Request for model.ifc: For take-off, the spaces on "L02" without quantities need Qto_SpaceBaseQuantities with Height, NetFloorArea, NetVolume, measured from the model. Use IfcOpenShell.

First a look at what the model holds.

```python
import ifcopenshell
import ifcopenshell.util.element
import ifcopenshell.util.unit

model = ifcopenshell.open("model.ifc")
print(model.schema)
for unit_type in ("LENGTHUNIT", "AREAUNIT", "VOLUMEUNIT"):
    print(unit_type, ifcopenshell.util.unit.calculate_unit_scale(model, unit_type))
storey = next(s for s in model.by_type("IfcBuildingStorey") if s.Name == "L02")
spaces = [e for e in ifcopenshell.util.element.get_decomposition(storey) if e.is_a("IfcSpace")]
for e in sorted(spaces, key=lambda e: e.id()):
    print(e.id(), e.is_a(), e.Name, list(ifcopenshell.util.element.get_psets(e, qtos_only=True)), sep=" | ")
```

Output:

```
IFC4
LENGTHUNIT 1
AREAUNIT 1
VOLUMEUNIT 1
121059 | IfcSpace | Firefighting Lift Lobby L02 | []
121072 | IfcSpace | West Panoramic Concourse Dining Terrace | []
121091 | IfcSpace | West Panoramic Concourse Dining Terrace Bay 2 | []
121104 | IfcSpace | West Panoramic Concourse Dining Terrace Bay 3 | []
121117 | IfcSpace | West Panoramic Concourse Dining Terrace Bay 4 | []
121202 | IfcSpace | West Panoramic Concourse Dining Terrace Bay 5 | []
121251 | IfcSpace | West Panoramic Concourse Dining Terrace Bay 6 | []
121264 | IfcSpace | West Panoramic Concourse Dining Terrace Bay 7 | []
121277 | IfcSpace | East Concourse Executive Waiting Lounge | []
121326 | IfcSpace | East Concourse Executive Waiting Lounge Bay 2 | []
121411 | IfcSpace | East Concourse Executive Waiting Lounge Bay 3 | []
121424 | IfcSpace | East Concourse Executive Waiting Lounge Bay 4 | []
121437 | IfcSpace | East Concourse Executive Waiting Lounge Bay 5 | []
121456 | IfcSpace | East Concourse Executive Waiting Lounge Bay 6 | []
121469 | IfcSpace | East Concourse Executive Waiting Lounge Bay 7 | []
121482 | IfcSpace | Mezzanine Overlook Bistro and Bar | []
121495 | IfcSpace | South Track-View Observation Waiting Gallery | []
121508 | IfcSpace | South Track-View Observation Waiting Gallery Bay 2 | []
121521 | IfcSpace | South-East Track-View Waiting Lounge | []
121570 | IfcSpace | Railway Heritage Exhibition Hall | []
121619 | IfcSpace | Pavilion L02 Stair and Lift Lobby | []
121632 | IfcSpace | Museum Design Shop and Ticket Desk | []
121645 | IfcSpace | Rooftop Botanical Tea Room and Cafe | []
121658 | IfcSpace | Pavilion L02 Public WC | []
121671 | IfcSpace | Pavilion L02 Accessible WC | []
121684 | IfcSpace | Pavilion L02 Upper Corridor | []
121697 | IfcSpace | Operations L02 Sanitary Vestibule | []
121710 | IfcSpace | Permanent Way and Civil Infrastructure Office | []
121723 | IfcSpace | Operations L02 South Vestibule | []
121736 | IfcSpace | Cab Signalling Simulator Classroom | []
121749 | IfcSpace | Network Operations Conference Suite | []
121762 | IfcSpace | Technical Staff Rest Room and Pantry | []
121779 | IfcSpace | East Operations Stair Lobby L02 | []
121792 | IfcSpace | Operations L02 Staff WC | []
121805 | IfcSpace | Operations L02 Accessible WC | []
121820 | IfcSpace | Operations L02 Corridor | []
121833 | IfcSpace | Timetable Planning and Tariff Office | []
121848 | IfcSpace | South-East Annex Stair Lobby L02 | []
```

```python
import ifcopenshell
import ifcopenshell.api.pset
import ifcopenshell.geom
import ifcopenshell.util.element
import ifcopenshell.util.shape
import ifcopenshell.util.unit

model = ifcopenshell.open("model.ifc")
unit_scale = ifcopenshell.util.unit.calculate_unit_scale(model)
area_scale = ifcopenshell.util.unit.calculate_unit_scale(model, "AREAUNIT")
volume_scale = ifcopenshell.util.unit.calculate_unit_scale(model, "VOLUMEUNIT")
settings = ifcopenshell.geom.settings()

storey = next(s for s in model.by_type("IfcBuildingStorey") if s.Name == "L02")
spaces = [e for e in ifcopenshell.util.element.get_decomposition(storey) if e.is_a("IfcSpace")]

for e in sorted(spaces, key=lambda e: e.id()):
    if ifcopenshell.util.element.get_psets(e, qtos_only=True, should_inherit=False):
        continue
    # Geometry comes back in metres, in the element's own axes.
    shape = ifcopenshell.geom.create_shape(settings, e)
    values = {
        "Height": ifcopenshell.util.shape.get_z(shape.geometry) / unit_scale,
        "NetFloorArea": ifcopenshell.util.shape.get_footprint_area(shape.geometry) / area_scale,
        "NetVolume": ifcopenshell.util.shape.get_volume(shape.geometry) / volume_scale,
    }
    qto = ifcopenshell.api.pset.add_qto(model, product=e, name="Qto_SpaceBaseQuantities")
    ifcopenshell.api.pset.edit_qto(model, qto=qto, properties=values)
    print(e.id(), {k: round(v, 3) for k, v in values.items()})

model.write("model_edited.ifc")
```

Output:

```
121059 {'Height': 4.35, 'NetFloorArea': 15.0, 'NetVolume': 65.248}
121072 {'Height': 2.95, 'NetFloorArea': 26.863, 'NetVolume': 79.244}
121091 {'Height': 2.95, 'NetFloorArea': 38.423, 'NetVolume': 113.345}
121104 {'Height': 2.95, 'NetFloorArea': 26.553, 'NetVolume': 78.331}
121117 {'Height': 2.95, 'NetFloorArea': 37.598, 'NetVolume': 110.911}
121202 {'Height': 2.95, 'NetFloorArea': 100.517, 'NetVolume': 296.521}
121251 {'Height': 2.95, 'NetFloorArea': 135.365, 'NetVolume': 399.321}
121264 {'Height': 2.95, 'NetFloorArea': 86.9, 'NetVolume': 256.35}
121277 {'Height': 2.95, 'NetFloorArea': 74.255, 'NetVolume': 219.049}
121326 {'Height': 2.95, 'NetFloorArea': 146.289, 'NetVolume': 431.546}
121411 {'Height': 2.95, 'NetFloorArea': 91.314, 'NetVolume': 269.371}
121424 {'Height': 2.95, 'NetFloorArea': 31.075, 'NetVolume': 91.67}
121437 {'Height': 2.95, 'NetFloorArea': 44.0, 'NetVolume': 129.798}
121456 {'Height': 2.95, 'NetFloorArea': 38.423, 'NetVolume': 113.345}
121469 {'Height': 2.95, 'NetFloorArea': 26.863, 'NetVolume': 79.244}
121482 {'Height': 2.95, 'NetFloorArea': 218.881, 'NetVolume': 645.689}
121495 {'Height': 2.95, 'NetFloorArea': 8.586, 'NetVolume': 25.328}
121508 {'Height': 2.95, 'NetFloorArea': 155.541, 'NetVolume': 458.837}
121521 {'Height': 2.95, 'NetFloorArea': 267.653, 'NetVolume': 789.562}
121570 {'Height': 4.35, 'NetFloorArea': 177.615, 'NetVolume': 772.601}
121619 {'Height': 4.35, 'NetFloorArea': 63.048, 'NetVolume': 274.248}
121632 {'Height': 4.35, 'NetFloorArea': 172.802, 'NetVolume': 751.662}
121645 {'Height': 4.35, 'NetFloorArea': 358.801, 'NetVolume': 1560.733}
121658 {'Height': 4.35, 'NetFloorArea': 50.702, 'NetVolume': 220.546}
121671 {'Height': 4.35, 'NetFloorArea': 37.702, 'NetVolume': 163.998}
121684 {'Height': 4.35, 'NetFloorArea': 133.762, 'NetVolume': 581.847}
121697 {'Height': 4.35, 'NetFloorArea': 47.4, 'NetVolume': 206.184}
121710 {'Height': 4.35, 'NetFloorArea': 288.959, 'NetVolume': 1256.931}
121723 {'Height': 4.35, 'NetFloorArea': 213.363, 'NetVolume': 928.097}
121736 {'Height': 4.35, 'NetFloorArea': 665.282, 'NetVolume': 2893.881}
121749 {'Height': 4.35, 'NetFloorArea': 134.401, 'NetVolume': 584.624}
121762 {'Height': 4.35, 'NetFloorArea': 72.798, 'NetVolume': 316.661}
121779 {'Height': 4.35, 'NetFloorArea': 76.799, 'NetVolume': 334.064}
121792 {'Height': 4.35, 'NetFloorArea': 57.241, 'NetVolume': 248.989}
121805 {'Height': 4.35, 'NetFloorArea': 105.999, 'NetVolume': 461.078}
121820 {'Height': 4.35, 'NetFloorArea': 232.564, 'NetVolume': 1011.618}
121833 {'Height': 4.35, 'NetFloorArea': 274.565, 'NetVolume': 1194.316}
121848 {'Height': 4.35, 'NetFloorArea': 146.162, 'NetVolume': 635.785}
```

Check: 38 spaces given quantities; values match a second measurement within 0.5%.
